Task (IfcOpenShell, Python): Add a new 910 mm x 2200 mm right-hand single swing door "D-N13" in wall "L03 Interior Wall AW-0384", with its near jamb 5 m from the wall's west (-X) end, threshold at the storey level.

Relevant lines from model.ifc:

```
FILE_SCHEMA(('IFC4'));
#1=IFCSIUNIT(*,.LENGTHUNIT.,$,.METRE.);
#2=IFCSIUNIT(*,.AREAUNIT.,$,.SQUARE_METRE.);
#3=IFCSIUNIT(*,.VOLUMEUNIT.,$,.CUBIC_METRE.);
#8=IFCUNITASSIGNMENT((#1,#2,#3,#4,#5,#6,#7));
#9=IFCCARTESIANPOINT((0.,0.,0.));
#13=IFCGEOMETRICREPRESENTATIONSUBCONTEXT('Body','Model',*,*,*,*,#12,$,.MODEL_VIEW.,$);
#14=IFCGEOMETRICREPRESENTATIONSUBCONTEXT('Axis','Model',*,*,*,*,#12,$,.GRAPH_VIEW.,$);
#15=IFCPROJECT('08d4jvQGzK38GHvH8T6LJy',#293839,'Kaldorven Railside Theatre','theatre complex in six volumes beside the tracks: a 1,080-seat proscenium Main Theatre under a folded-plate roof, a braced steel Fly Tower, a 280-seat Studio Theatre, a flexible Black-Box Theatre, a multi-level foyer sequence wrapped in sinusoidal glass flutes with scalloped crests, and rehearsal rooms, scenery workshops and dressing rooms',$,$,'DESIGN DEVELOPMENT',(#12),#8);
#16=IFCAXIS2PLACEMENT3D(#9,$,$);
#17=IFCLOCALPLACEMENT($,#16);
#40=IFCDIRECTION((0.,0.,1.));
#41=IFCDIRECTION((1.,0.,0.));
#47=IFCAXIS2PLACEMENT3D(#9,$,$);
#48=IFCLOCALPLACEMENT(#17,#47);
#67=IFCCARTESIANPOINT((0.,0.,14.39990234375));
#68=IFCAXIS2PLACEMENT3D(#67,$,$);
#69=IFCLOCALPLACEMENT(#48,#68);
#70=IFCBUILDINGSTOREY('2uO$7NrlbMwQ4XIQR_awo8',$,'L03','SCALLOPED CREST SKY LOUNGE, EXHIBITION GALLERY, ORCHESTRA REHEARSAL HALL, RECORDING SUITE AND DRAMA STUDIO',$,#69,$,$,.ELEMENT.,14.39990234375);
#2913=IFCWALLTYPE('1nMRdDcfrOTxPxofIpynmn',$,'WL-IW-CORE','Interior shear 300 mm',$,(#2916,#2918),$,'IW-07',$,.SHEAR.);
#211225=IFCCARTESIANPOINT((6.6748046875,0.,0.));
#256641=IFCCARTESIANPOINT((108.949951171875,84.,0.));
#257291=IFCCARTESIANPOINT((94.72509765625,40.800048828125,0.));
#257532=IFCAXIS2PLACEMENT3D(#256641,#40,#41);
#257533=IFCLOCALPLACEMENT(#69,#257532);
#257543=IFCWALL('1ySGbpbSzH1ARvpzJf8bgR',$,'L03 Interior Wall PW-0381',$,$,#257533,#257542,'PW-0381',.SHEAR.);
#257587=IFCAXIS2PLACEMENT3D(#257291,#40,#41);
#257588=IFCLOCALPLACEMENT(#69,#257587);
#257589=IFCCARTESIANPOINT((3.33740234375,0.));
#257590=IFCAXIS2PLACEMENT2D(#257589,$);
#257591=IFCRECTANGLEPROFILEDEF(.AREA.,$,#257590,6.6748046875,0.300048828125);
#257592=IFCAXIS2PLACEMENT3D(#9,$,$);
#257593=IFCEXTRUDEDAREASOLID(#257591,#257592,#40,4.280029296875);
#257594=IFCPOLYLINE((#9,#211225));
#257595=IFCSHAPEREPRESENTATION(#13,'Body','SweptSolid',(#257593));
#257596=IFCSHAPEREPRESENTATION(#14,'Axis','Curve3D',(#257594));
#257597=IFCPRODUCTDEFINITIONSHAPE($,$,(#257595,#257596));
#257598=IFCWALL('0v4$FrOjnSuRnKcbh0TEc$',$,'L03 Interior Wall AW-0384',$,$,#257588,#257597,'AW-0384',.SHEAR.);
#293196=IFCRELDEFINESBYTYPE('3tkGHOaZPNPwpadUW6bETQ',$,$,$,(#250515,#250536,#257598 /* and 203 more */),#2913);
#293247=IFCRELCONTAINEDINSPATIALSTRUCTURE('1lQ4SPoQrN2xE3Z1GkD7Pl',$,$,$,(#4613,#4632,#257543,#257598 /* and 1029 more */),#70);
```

```python
import numpy as np
import ifcopenshell
import ifcopenshell.api.feature
import ifcopenshell.api.geometry
import ifcopenshell.api.root
import ifcopenshell.api.spatial
import ifcopenshell.geom
import ifcopenshell.util.element
import ifcopenshell.util.placement
import ifcopenshell.util.representation
import ifcopenshell.util.shape
import ifcopenshell.util.unit

model = ifcopenshell.open("model.ifc")
unit_scale = ifcopenshell.util.unit.calculate_unit_scale(model)
settings = ifcopenshell.geom.settings()


def volume(element):
    """Net volume in cubic metres, openings subtracted."""
    shape = ifcopenshell.geom.create_shape(settings, element)
    return ifcopenshell.util.shape.get_volume(shape.geometry)


wall = model.by_id(257598)
storey = ifcopenshell.util.element.get_container(wall, ifc_class="IfcBuildingStorey")
context = ifcopenshell.util.representation.get_context(model, "Model", "Body", "MODEL_VIEW")
before = volume(wall)

width, height, from_end, sill = 0.91, 2.2, 5, 0.0  # metres

# The wall runs along its own X axis, and the end named is its -X end.
wall_shape = ifcopenshell.geom.create_shape(settings, wall)
x, y, z = ifcopenshell.util.shape.get_vertices(wall_shape.geometry).T
start = x.min() + from_end
face, thickness = float(y.min()), float(y.max() - y.min())
wall_matrix = ifcopenshell.util.placement.get_local_placement(wall.ObjectPlacement)
level = ifcopenshell.util.placement.get_local_placement(storey.ObjectPlacement)[2, 3]


def in_wall(x, y):
    """Placement at x, y metres in the wall's axes, at sill height."""
    matrix = wall_matrix.copy()
    matrix[:, 3] = wall_matrix @ np.array([x / unit_scale, y / unit_scale, 0.0, 1.0])
    matrix[2, 3] = level + sill / unit_scale
    return matrix


# Opening: a box that overshoots both wall faces by 50 mm.
opening = ifcopenshell.api.root.create_entity(model, ifc_class="IfcOpeningElement", predefined_type="OPENING")
box = ifcopenshell.api.geometry.add_wall_representation(
    model, context=context, length=width, height=height, thickness=thickness + 0.1
)
ifcopenshell.api.geometry.assign_representation(model, product=opening, representation=box)
ifcopenshell.api.geometry.edit_object_placement(model, product=opening, matrix=in_wall(start, face - 0.05), is_si=False)
ifcopenshell.api.feature.add_feature(model, feature=opening, element=wall)

door = ifcopenshell.api.root.create_entity(model, ifc_class="IfcDoor", name="D-N13", predefined_type="DOOR")
door.OverallWidth, door.OverallHeight = width / unit_scale, height / unit_scale
door.OperationType = "SINGLE_SWING_RIGHT"
body = ifcopenshell.api.geometry.add_door_representation(
    model,
    context=context,
    overall_width=door.OverallWidth,
    overall_height=door.OverallHeight,
    operation_type="SINGLE_SWING_RIGHT",
    lining_properties={"LiningDepth": thickness / unit_scale, "ThresholdDepth": thickness / unit_scale},
)
ifcopenshell.api.geometry.assign_representation(model, product=door, representation=body)
ifcopenshell.api.spatial.assign_container(model, products=[door], relating_structure=storey)
ifcopenshell.api.feature.add_filling(model, opening=opening, element=door)

# The lining spans the wall, so the door starts at the wall face.
ifcopenshell.api.geometry.edit_object_placement(model, product=door, matrix=in_wall(start, face), is_si=False)

after = volume(wall)

print(f"wall volume {before:.3f} -> {after:.3f} m3")

model.write("model_updated.ifc")
```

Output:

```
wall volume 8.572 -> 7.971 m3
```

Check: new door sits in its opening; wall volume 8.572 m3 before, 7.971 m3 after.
